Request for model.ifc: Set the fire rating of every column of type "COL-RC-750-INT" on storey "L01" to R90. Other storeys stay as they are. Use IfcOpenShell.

First a look at what the model holds.

```python
import ifcopenshell
import ifcopenshell.util.element

model = ifcopenshell.open("model.ifc")
print(model.schema)
storey = next(s for s in model.by_type("IfcBuildingStorey") if s.Name == "L01")
columns = [e for e in ifcopenshell.util.element.get_decomposition(storey) if e.is_a("IfcColumn")]
seen = {}
for e in columns:
    element_type = ifcopenshell.util.element.get_type(e)
    key = (element_type.Name if element_type != e and element_type else None, ifcopenshell.util.element.get_pset(e, "Pset_ColumnCommon", "FireRating"))
    seen[key] = seen.get(key, 0) + 1
for (name, value), count in sorted(seen.items(), key=str):
    print(count, "x", name, "|", value)
```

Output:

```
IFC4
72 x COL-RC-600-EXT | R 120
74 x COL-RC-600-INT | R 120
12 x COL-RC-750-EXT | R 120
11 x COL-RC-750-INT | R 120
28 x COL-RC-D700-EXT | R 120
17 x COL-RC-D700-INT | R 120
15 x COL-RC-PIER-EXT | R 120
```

```python
import ifcopenshell
import ifcopenshell.api.pset
import ifcopenshell.util.element

model = ifcopenshell.open("model.ifc")

storey = next(s for s in model.by_type("IfcBuildingStorey") if s.Name == "L01")
columns = [e for e in ifcopenshell.util.element.get_decomposition(storey) if e.is_a("IfcColumn")]

count = 0
for e in columns:
    element_type = ifcopenshell.util.element.get_type(e)
    if element_type in (None, e) or element_type.Name != "COL-RC-750-INT":
        continue
    # add_pset returns the element's existing set when there is one.
    pset = ifcopenshell.api.pset.add_pset(model, product=e, name="Pset_ColumnCommon")
    ifcopenshell.api.pset.edit_pset(model, pset=pset, properties={"FireRating": "R90"})
    count += 1

print(count, "columns updated")

model.write("model_v2.ifc")
```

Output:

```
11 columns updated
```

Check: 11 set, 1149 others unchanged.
